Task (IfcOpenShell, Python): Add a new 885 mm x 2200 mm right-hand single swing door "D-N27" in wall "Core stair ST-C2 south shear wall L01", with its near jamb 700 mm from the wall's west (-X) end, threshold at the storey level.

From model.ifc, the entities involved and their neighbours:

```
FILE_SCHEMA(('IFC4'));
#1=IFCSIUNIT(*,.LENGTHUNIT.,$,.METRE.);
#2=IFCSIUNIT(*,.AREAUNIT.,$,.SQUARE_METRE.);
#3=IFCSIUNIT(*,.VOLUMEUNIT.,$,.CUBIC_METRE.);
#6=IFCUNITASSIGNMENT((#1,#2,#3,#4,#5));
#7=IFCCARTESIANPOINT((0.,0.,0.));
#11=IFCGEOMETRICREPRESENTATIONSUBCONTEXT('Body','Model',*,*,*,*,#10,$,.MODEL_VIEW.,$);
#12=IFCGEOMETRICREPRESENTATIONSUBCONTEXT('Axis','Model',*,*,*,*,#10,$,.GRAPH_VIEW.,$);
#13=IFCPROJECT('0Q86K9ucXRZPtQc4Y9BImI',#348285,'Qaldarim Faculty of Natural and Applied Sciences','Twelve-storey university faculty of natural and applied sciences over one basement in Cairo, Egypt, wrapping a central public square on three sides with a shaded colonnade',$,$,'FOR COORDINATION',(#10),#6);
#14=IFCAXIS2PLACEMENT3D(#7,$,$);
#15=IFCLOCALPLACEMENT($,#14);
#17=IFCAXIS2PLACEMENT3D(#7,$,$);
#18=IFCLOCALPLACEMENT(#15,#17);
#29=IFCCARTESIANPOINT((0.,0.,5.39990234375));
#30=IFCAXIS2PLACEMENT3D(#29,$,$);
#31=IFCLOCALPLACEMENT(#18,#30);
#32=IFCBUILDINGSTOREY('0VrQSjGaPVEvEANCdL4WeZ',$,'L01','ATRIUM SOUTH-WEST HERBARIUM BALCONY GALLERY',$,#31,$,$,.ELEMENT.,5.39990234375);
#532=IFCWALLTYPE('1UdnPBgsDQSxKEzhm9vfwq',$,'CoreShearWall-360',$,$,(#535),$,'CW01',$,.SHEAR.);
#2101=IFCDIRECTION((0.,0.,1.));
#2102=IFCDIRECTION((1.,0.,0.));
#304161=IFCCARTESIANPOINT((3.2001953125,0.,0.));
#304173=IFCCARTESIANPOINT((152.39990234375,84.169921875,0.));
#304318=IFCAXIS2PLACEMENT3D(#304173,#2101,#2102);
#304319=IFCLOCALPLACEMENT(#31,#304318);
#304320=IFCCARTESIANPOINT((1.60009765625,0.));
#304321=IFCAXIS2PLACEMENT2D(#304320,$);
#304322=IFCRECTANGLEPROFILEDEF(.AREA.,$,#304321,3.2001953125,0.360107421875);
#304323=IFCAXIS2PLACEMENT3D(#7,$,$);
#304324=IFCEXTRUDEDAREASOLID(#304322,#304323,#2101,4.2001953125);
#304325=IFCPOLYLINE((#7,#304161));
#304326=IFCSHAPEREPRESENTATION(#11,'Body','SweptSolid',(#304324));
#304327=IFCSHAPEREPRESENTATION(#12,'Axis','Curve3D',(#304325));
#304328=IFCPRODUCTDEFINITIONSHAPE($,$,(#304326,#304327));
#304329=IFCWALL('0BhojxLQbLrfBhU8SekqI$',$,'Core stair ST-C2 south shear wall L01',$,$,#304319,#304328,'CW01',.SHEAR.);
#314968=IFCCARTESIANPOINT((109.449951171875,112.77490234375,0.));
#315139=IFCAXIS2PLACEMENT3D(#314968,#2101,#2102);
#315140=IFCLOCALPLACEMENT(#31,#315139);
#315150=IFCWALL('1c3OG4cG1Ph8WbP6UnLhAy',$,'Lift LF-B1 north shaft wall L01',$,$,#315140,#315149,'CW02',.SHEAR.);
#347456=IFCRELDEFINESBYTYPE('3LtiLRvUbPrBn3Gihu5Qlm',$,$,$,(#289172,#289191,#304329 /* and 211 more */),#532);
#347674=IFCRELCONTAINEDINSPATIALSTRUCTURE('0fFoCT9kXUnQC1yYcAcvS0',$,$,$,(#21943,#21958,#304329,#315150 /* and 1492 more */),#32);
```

```python
import numpy as np
import ifcopenshell
import ifcopenshell.api.feature
import ifcopenshell.api.geometry
import ifcopenshell.api.root
import ifcopenshell.api.spatial
import ifcopenshell.geom
import ifcopenshell.util.element
import ifcopenshell.util.placement
import ifcopenshell.util.representation
import ifcopenshell.util.shape
import ifcopenshell.util.unit

model = ifcopenshell.open("model.ifc")
unit_scale = ifcopenshell.util.unit.calculate_unit_scale(model)
settings = ifcopenshell.geom.settings()


def volume(element):
    """Net volume in cubic metres, openings subtracted."""
    shape = ifcopenshell.geom.create_shape(settings, element)
    return ifcopenshell.util.shape.get_volume(shape.geometry)


wall = model.by_guid("0BhojxLQbLrfBhU8SekqI$")
storey = ifcopenshell.util.element.get_container(wall, ifc_class="IfcBuildingStorey")
context = ifcopenshell.util.representation.get_context(model, "Model", "Body", "MODEL_VIEW")
before = volume(wall)

width, height, from_end, sill = 0.885, 2.2, 0.7, 0.0  # metres

# The wall runs along its own X axis, and the end named is its -X end.
wall_shape = ifcopenshell.geom.create_shape(settings, wall)
x, y, z = ifcopenshell.util.shape.get_vertices(wall_shape.geometry).T
start = x.min() + from_end
face, thickness = float(y.min()), float(y.max() - y.min())
wall_matrix = ifcopenshell.util.placement.get_local_placement(wall.ObjectPlacement)
level = ifcopenshell.util.placement.get_local_placement(storey.ObjectPlacement)[2, 3]


def in_wall(x, y):
    """Placement at x, y metres in the wall's axes, at sill height."""
    matrix = wall_matrix.copy()
    matrix[:, 3] = wall_matrix @ np.array([x / unit_scale, y / unit_scale, 0.0, 1.0])
    matrix[2, 3] = level + sill / unit_scale
    return matrix


# Opening: a box that overshoots both wall faces by 50 mm.
opening = ifcopenshell.api.root.create_entity(model, ifc_class="IfcOpeningElement", predefined_type="OPENING")
box = ifcopenshell.api.geometry.add_wall_representation(
    model, context=context, length=width, height=height, thickness=thickness + 0.1
)
ifcopenshell.api.geometry.assign_representation(model, product=opening, representation=box)
ifcopenshell.api.geometry.edit_object_placement(model, product=opening, matrix=in_wall(start, face - 0.05), is_si=False)
ifcopenshell.api.feature.add_feature(model, feature=opening, element=wall)

door = ifcopenshell.api.root.create_entity(model, ifc_class="IfcDoor", name="D-N27", predefined_type="DOOR")
door.OverallWidth, door.OverallHeight = width / unit_scale, height / unit_scale
door.OperationType = "SINGLE_SWING_RIGHT"
body = ifcopenshell.api.geometry.add_door_representation(
    model,
    context=context,
    overall_width=door.OverallWidth,
    overall_height=door.OverallHeight,
    operation_type="SINGLE_SWING_RIGHT",
    lining_properties={"LiningDepth": thickness / unit_scale, "ThresholdDepth": thickness / unit_scale},
)
ifcopenshell.api.geometry.assign_representation(model, product=door, representation=body)
ifcopenshell.api.spatial.assign_container(model, products=[door], relating_structure=storey)
ifcopenshell.api.feature.add_filling(model, opening=opening, element=door)

# The lining spans the wall, so the door starts at the wall face.
ifcopenshell.api.geometry.edit_object_placement(model, product=door, matrix=in_wall(start, face), is_si=False)

after = volume(wall)

print(f"wall volume {before:.3f} -> {after:.3f} m3")

model.write("model_edited.ifc")
```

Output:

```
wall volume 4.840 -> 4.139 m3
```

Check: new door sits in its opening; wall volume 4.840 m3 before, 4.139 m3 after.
